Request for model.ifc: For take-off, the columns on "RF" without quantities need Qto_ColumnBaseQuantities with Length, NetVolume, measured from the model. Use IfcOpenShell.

First a look at what the model holds.

```python
import ifcopenshell
import ifcopenshell.util.element
import ifcopenshell.util.unit

model = ifcopenshell.open("model.ifc")
print(model.schema)
for unit_type in ("LENGTHUNIT", "AREAUNIT", "VOLUMEUNIT"):
    print(unit_type, ifcopenshell.util.unit.calculate_unit_scale(model, unit_type))
storey = next(s for s in model.by_type("IfcBuildingStorey") if s.Name == "RF")
columns = [e for e in ifcopenshell.util.element.get_decomposition(storey) if e.is_a("IfcColumn")]
for e in sorted(columns, key=lambda e: e.id()):
    print(e.id(), e.is_a(), e.Name, list(ifcopenshell.util.element.get_psets(e, qtos_only=True)), sep=" | ")
```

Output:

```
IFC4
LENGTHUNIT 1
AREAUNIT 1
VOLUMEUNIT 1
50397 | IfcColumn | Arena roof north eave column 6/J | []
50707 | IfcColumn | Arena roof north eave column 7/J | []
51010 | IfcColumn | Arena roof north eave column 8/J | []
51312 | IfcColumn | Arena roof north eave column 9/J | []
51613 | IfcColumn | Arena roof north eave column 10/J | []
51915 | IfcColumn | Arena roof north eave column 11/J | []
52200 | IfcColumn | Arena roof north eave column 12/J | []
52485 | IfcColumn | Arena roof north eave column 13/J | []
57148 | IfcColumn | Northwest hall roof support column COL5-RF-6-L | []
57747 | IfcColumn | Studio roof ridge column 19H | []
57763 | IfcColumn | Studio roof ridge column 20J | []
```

```python
import ifcopenshell
import ifcopenshell.api.pset
import ifcopenshell.geom
import ifcopenshell.util.element
import ifcopenshell.util.shape
import ifcopenshell.util.unit

model = ifcopenshell.open("model.ifc")
unit_scale = ifcopenshell.util.unit.calculate_unit_scale(model)
volume_scale = ifcopenshell.util.unit.calculate_unit_scale(model, "VOLUMEUNIT")
settings = ifcopenshell.geom.settings()

storey = next(s for s in model.by_type("IfcBuildingStorey") if s.Name == "RF")
columns = [e for e in ifcopenshell.util.element.get_decomposition(storey) if e.is_a("IfcColumn")]

for e in sorted(columns, key=lambda e: e.id()):
    if ifcopenshell.util.element.get_psets(e, qtos_only=True, should_inherit=False):
        continue
    # Geometry comes back in metres, in the element's own axes.
    shape = ifcopenshell.geom.create_shape(settings, e)
    values = {
        "Length": ifcopenshell.util.shape.get_z(shape.geometry) / unit_scale,
        "NetVolume": ifcopenshell.util.shape.get_volume(shape.geometry) / volume_scale,
    }
    qto = ifcopenshell.api.pset.add_qto(model, product=e, name="Qto_ColumnBaseQuantities")
    ifcopenshell.api.pset.edit_qto(model, qto=qto, properties=values)
    print(e.id(), {k: round(v, 3) for k, v in values.items()})

model.write("model-out.ifc")
```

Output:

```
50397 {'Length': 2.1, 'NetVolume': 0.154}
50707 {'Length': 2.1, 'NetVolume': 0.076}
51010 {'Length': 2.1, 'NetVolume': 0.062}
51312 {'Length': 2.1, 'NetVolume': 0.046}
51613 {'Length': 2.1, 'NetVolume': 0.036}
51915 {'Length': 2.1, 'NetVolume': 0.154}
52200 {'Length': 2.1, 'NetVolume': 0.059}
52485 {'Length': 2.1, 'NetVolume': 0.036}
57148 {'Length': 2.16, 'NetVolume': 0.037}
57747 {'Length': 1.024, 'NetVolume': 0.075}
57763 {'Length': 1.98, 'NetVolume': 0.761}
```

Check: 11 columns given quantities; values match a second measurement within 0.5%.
